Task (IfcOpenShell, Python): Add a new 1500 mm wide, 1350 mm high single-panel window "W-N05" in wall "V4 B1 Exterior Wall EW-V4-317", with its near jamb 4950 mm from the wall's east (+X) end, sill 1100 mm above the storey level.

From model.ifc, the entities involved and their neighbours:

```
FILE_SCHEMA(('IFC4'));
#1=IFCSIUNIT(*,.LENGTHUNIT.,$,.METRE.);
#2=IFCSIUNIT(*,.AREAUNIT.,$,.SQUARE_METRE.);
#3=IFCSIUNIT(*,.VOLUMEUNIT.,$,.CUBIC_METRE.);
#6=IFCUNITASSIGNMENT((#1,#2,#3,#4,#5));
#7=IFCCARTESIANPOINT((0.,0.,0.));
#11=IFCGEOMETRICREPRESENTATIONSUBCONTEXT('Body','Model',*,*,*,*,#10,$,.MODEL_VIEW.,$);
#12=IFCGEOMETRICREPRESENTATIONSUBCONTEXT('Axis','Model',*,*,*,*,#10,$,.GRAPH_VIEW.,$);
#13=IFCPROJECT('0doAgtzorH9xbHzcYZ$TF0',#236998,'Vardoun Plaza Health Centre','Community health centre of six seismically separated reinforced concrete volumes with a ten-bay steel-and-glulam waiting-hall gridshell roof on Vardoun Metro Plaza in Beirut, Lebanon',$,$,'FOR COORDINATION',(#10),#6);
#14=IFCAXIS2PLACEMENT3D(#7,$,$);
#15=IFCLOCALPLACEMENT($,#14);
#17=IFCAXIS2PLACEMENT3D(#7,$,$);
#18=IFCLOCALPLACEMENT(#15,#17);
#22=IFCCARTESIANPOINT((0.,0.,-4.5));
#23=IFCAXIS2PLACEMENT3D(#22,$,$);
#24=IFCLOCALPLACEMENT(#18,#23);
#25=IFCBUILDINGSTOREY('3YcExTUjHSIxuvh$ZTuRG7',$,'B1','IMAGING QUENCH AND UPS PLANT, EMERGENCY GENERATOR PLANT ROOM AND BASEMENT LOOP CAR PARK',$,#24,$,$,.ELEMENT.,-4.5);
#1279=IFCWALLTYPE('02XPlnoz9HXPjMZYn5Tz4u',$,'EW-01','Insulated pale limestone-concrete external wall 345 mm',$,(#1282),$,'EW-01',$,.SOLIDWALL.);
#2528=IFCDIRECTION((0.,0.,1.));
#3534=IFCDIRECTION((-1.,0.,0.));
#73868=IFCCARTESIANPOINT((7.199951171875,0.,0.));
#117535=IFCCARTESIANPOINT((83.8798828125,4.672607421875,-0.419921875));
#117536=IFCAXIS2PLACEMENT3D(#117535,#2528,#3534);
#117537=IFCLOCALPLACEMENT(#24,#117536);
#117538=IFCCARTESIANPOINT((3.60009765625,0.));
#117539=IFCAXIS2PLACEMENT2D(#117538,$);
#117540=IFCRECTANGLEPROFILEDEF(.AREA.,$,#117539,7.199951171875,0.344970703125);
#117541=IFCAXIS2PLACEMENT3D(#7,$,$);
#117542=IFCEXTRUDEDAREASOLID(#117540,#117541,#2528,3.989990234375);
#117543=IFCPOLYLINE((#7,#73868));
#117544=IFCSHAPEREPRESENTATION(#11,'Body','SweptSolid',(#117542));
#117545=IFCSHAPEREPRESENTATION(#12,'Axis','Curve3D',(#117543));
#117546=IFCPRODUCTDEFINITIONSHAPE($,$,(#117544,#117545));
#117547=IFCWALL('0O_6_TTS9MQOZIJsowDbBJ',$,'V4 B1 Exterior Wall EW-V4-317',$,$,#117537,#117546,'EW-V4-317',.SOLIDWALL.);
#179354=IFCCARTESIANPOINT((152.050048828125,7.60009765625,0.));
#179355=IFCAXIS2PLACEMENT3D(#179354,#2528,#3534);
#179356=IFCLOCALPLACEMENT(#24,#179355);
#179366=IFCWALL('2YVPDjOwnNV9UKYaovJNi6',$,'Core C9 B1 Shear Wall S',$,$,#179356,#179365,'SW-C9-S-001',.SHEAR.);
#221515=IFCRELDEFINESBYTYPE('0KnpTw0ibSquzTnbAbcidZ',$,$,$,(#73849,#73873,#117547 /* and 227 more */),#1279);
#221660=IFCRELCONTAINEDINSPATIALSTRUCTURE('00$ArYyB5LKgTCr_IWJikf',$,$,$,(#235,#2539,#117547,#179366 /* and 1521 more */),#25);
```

```python
import numpy as np
import ifcopenshell
import ifcopenshell.api.feature
import ifcopenshell.api.geometry
import ifcopenshell.api.root
import ifcopenshell.api.spatial
import ifcopenshell.geom
import ifcopenshell.util.element
import ifcopenshell.util.placement
import ifcopenshell.util.representation
import ifcopenshell.util.shape
import ifcopenshell.util.unit

model = ifcopenshell.open("model.ifc")
unit_scale = ifcopenshell.util.unit.calculate_unit_scale(model)
settings = ifcopenshell.geom.settings()


def volume(element):
    """Net volume in cubic metres, openings subtracted."""
    shape = ifcopenshell.geom.create_shape(settings, element)
    return ifcopenshell.util.shape.get_volume(shape.geometry)


wall = model.by_guid("0O_6_TTS9MQOZIJsowDbBJ")
storey = ifcopenshell.util.element.get_container(wall, ifc_class="IfcBuildingStorey")
context = ifcopenshell.util.representation.get_context(model, "Model", "Body", "MODEL_VIEW")
before = volume(wall)

width, height, from_end, sill = 1.5, 1.35, 4.95, 1.1  # metres

# The wall runs along its own X axis, and the end named is its -X end.
wall_shape = ifcopenshell.geom.create_shape(settings, wall)
x, y, z = ifcopenshell.util.shape.get_vertices(wall_shape.geometry).T
start = x.min() + from_end
face, thickness = float(y.min()), float(y.max() - y.min())
wall_matrix = ifcopenshell.util.placement.get_local_placement(wall.ObjectPlacement)
level = ifcopenshell.util.placement.get_local_placement(storey.ObjectPlacement)[2, 3]


def in_wall(x, y):
    """Placement at x, y metres in the wall's axes, at sill height."""
    matrix = wall_matrix.copy()
    matrix[:, 3] = wall_matrix @ np.array([x / unit_scale, y / unit_scale, 0.0, 1.0])
    matrix[2, 3] = level + sill / unit_scale
    return matrix


# Opening: a box that overshoots both wall faces by 50 mm.
opening = ifcopenshell.api.root.create_entity(model, ifc_class="IfcOpeningElement", predefined_type="OPENING")
box = ifcopenshell.api.geometry.add_wall_representation(
    model, context=context, length=width, height=height, thickness=thickness + 0.1
)
ifcopenshell.api.geometry.assign_representation(model, product=opening, representation=box)
ifcopenshell.api.geometry.edit_object_placement(model, product=opening, matrix=in_wall(start, face - 0.05), is_si=False)
ifcopenshell.api.feature.add_feature(model, feature=opening, element=wall)

window = ifcopenshell.api.root.create_entity(model, ifc_class="IfcWindow", name="W-N05", predefined_type="WINDOW")
window.OverallWidth, window.OverallHeight = width / unit_scale, height / unit_scale
window.PartitioningType = "SINGLE_PANEL"
body = ifcopenshell.api.geometry.add_window_representation(
    model,
    context=context,
    overall_width=window.OverallWidth,
    overall_height=window.OverallHeight,
    partition_type="SINGLE_PANEL",
)
ifcopenshell.api.geometry.assign_representation(model, product=window, representation=body)
ifcopenshell.api.spatial.assign_container(model, products=[window], relating_structure=storey)
ifcopenshell.api.feature.add_filling(model, opening=opening, element=window)

# Centre the window in the wall's thickness.
ifcopenshell.api.geometry.edit_object_placement(model, product=window, matrix=in_wall(start, face), is_si=False)
window_shape = ifcopenshell.geom.create_shape(settings, window)
depth = ifcopenshell.util.shape.get_vertices(window_shape.geometry)[:, 1]
offset = face + thickness / 2 - (depth.min() + depth.max()) / 2
ifcopenshell.api.geometry.edit_object_placement(model, product=window, matrix=in_wall(start, offset), is_si=False)

after = volume(wall)

print(f"wall volume {before:.3f} -> {after:.3f} m3")

model.write("model_updated.ifc")
```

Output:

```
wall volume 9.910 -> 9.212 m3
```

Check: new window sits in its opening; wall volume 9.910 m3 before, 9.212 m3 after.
